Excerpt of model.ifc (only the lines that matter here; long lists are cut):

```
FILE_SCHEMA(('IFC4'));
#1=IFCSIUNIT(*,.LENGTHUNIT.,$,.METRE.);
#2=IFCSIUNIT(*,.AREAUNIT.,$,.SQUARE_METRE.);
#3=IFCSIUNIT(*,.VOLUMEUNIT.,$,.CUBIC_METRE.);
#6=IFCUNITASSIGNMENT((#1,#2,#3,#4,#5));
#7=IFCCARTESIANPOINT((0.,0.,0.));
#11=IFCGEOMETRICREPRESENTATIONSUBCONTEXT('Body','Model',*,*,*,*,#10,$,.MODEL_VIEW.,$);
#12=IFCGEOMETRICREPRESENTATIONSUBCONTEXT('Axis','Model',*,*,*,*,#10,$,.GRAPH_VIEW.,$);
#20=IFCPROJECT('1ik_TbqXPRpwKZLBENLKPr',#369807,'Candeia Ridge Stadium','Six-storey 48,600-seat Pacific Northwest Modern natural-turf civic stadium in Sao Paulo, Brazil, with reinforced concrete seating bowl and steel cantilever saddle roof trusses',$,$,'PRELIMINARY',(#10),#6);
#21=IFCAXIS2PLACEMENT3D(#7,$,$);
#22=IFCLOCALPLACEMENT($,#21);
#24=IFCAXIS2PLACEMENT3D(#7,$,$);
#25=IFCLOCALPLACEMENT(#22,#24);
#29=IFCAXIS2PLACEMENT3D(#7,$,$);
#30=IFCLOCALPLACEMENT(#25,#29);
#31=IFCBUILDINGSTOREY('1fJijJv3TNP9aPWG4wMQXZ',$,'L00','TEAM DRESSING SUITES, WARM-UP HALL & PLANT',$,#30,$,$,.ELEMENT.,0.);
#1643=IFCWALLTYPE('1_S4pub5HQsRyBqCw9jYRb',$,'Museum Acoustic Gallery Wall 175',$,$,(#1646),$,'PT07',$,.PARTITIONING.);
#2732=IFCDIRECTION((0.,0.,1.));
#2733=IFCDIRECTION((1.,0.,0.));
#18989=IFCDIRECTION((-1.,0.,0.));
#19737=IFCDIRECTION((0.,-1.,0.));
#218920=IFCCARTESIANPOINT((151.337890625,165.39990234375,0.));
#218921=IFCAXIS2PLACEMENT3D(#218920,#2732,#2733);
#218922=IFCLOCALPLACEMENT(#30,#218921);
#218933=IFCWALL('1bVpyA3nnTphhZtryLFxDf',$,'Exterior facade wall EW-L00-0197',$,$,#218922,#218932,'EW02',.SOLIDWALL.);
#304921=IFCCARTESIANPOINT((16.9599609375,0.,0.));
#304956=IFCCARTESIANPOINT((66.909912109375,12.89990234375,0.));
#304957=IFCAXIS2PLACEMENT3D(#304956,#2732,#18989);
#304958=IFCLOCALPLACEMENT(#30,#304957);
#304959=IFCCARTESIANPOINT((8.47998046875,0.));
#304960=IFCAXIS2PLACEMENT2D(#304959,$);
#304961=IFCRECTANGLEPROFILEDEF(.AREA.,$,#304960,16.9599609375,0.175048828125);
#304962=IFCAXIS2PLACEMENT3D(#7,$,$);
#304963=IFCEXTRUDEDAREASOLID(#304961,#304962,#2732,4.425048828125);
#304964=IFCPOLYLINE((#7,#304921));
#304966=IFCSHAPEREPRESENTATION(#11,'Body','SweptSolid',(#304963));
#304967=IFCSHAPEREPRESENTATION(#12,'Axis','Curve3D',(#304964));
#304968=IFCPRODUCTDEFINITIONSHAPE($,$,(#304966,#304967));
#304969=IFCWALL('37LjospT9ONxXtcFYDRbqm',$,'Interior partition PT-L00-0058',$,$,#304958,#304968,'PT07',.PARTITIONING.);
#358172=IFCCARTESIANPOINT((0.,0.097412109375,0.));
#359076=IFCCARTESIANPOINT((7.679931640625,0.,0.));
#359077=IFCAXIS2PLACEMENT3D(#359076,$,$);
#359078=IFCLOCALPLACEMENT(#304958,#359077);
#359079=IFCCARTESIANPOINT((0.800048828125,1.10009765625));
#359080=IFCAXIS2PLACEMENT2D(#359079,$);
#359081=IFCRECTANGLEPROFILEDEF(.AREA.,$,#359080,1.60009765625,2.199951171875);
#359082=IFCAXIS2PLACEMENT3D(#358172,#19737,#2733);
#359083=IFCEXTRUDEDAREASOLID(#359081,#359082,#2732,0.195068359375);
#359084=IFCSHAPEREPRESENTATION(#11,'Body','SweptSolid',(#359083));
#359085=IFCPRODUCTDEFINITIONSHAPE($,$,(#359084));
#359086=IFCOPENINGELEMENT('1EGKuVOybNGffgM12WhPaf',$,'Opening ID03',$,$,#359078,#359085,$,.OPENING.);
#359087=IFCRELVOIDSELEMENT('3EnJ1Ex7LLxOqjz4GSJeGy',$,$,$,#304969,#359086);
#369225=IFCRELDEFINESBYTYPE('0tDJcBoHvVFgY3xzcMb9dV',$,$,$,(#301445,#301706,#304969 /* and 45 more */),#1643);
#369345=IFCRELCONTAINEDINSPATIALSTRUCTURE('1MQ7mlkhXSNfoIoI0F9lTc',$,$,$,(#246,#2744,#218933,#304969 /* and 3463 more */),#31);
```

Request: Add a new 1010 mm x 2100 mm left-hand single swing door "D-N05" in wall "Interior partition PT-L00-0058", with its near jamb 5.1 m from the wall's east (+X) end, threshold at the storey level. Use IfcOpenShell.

```python
import numpy as np
import ifcopenshell
import ifcopenshell.api.feature
import ifcopenshell.api.geometry
import ifcopenshell.api.root
import ifcopenshell.api.spatial
import ifcopenshell.geom
import ifcopenshell.util.element
import ifcopenshell.util.placement
import ifcopenshell.util.representation
import ifcopenshell.util.shape
import ifcopenshell.util.unit

model = ifcopenshell.open("model.ifc")
unit_scale = ifcopenshell.util.unit.calculate_unit_scale(model)
settings = ifcopenshell.geom.settings()


def volume(element):
    """Net volume in cubic metres, openings subtracted."""
    shape = ifcopenshell.geom.create_shape(settings, element)
    return ifcopenshell.util.shape.get_volume(shape.geometry)


wall = model.by_guid("37LjospT9ONxXtcFYDRbqm")
storey = ifcopenshell.util.element.get_container(wall, ifc_class="IfcBuildingStorey")
context = ifcopenshell.util.representation.get_context(model, "Model", "Body", "MODEL_VIEW")
before = volume(wall)

width, height, from_end, sill = 1.01, 2.1, 5.1, 0.0  # metres

# The wall runs along its own X axis, and the end named is its -X end.
wall_shape = ifcopenshell.geom.create_shape(settings, wall)
x, y, z = ifcopenshell.util.shape.get_vertices(wall_shape.geometry).T
start = x.min() + from_end
face, thickness = float(y.min()), float(y.max() - y.min())
wall_matrix = ifcopenshell.util.placement.get_local_placement(wall.ObjectPlacement)
level = ifcopenshell.util.placement.get_local_placement(storey.ObjectPlacement)[2, 3]


def in_wall(x, y):
    """Placement at x, y metres in the wall's axes, at sill height."""
    matrix = wall_matrix.copy()
    matrix[:, 3] = wall_matrix @ np.array([x / unit_scale, y / unit_scale, 0.0, 1.0])
    matrix[2, 3] = level + sill / unit_scale
    return matrix


# Opening: a box that overshoots both wall faces by 50 mm.
opening = ifcopenshell.api.root.create_entity(model, ifc_class="IfcOpeningElement", predefined_type="OPENING")
box = ifcopenshell.api.geometry.add_wall_representation(
    model, context=context, length=width, height=height, thickness=thickness + 0.1
)
ifcopenshell.api.geometry.assign_representation(model, product=opening, representation=box)
ifcopenshell.api.geometry.edit_object_placement(model, product=opening, matrix=in_wall(start, face - 0.05), is_si=False)
ifcopenshell.api.feature.add_feature(model, feature=opening, element=wall)

door = ifcopenshell.api.root.create_entity(model, ifc_class="IfcDoor", name="D-N05", predefined_type="DOOR")
door.OverallWidth, door.OverallHeight = width / unit_scale, height / unit_scale
door.OperationType = "SINGLE_SWING_LEFT"
body = ifcopenshell.api.geometry.add_door_representation(
    model,
    context=context,
    overall_width=door.OverallWidth,
    overall_height=door.OverallHeight,
    operation_type="SINGLE_SWING_LEFT",
    lining_properties={"LiningDepth": thickness / unit_scale, "ThresholdDepth": thickness / unit_scale},
)
ifcopenshell.api.geometry.assign_representation(model, product=door, representation=body)
ifcopenshell.api.spatial.assign_container(model, products=[door], relating_structure=storey)
ifcopenshell.api.feature.add_filling(model, opening=opening, element=door)

# The lining spans the wall, so the door starts at the wall face.
ifcopenshell.api.geometry.edit_object_placement(model, product=door, matrix=in_wall(start, face), is_si=False)

after = volume(wall)

print(f"wall volume {before:.3f} -> {after:.3f} m3")

model.write("model_rev.ifc")
```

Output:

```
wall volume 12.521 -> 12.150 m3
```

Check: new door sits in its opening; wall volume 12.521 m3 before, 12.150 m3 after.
